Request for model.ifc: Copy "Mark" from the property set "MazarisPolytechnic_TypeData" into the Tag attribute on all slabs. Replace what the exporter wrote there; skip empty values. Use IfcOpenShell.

First a look at what the model holds.

```python
import ifcopenshell
import ifcopenshell.util.element

model = ifcopenshell.open("model.ifc")
print(model.schema)
slabs = model.by_type("IfcSlab")
print(len(slabs), "slabs")
for e in slabs[:8]:
    source = ifcopenshell.util.element.get_pset(e, "MazarisPolytechnic_TypeData", "Mark")
    target = e.Tag
    print(e.id(), repr(source), repr(target), sep=" | ")
```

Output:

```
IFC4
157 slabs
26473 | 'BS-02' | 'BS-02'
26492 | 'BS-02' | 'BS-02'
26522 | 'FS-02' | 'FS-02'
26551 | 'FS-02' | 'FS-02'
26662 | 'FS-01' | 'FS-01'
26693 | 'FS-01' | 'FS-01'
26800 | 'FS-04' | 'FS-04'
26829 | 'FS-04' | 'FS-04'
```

```python
import ifcopenshell
import ifcopenshell.util.element

model = ifcopenshell.open("model.ifc")

count = 0
for e in model.by_type("IfcSlab"):
    value = ifcopenshell.util.element.get_pset(e, "MazarisPolytechnic_TypeData", "Mark")
    current = e.Tag
    if not value or not value.strip() or current == value:
        continue
    e.Tag = value
    count += 1

print(count, "slabs updated")

model.write("model-out.ifc")
```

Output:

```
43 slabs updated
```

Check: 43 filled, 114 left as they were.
